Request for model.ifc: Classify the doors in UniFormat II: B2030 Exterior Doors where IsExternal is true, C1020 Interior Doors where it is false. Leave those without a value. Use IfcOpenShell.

First a look at what the model holds.

```python
import ifcopenshell
import ifcopenshell.util.element

model = ifcopenshell.open("model.ifc")
print(model.schema)
print("classifications:", [c.Name for c in model.by_type("IfcClassification")])
values = [ifcopenshell.util.element.get_pset(e, "Pset_DoorCommon", "IsExternal") for e in model.by_type("IfcDoor")]
for value in (True, False, None):
    print("IsExternal", value, values.count(value))
```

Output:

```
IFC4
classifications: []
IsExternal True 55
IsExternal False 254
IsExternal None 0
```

```python
import ifcopenshell
import ifcopenshell.api.classification
import ifcopenshell.util.element

model = ifcopenshell.open("model.ifc")

system = ifcopenshell.api.classification.add_classification(model, classification="UniFormat II")

doors = model.by_type("IfcDoor")
external = {e: ifcopenshell.util.element.get_pset(e, "Pset_DoorCommon", "IsExternal") for e in doors}
for flag, code, name in ((True, "B2030", "Exterior Doors"), (False, "C1020", "Interior Doors")):
    products = [e for e in doors if external[e] is flag]
    ifcopenshell.api.classification.add_reference(
        model, products=products, classification=system, identification=code, name=name
    )
    print(code, len(products))

model.write("model_edited.ifc")
```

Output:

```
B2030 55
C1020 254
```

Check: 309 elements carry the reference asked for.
